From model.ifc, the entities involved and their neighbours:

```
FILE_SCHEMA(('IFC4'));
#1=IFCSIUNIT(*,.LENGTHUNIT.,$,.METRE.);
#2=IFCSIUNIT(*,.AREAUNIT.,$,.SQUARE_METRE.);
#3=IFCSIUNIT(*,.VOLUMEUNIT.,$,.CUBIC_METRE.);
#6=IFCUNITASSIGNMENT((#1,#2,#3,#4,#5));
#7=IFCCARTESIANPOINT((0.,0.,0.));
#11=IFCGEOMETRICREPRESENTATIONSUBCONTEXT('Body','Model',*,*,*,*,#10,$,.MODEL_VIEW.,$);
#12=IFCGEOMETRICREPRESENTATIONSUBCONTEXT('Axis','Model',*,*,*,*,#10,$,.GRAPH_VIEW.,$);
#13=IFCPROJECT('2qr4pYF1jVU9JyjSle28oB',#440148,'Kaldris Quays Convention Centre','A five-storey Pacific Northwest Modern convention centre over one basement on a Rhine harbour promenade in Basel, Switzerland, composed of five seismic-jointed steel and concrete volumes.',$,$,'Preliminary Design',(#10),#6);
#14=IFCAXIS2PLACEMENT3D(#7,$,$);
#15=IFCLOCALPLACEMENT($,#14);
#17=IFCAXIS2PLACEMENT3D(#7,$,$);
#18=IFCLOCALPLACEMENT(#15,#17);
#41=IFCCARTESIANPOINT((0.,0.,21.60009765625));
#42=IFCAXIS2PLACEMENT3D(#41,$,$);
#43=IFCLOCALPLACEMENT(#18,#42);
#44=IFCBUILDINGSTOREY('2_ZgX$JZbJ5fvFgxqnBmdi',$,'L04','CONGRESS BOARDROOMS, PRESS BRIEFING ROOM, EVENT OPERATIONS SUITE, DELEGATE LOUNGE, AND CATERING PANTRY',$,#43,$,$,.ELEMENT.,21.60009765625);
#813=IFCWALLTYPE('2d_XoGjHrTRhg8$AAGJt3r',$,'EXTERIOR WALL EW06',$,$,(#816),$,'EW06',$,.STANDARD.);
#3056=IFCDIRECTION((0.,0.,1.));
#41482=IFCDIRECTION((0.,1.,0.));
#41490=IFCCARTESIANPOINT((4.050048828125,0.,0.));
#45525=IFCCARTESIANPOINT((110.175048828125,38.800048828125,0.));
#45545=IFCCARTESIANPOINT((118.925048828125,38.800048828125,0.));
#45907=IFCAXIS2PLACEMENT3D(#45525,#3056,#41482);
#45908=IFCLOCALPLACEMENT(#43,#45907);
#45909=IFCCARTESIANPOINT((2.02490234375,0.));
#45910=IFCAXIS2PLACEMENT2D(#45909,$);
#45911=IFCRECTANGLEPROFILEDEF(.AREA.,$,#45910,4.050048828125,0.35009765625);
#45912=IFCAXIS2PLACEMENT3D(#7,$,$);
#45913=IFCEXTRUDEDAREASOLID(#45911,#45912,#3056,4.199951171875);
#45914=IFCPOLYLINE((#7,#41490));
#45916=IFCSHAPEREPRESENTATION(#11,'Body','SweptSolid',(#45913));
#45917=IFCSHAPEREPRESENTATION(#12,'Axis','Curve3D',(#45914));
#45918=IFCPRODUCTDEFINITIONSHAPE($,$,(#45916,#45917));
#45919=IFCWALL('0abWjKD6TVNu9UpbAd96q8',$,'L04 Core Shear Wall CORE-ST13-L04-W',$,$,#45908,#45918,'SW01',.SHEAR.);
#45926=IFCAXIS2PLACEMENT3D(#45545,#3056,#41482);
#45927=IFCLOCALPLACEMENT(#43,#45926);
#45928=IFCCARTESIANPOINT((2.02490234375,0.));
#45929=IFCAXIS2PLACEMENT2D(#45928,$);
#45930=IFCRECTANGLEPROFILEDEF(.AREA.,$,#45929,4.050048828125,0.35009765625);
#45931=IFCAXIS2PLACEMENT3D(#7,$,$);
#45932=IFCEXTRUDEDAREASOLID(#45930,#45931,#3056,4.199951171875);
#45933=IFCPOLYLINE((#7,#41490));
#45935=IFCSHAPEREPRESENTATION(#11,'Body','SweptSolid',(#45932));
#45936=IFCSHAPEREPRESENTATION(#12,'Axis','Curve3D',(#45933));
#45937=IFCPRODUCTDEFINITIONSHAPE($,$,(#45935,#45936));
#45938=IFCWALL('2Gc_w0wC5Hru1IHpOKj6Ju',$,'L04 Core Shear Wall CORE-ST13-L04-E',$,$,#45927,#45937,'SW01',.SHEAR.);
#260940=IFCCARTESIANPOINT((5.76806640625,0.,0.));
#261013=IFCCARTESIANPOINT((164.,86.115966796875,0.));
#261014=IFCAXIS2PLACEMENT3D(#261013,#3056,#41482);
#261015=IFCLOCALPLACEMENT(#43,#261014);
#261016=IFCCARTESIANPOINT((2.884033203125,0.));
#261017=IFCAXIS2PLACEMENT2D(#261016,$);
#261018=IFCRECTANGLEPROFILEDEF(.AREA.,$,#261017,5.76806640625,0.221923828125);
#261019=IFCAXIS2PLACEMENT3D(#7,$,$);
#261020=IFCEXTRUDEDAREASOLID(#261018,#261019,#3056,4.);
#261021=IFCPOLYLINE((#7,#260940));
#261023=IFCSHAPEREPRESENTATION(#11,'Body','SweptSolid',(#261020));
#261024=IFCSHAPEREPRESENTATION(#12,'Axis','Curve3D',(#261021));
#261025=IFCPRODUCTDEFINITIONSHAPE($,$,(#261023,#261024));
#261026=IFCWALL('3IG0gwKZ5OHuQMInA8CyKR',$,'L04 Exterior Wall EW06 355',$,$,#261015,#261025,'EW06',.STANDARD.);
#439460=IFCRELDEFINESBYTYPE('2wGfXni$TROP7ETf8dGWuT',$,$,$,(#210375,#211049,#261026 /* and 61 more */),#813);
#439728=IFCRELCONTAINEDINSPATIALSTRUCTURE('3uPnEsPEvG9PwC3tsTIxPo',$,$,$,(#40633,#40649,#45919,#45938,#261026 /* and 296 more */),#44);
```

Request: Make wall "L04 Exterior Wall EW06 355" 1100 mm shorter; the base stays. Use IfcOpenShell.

```python
import ifcopenshell
import ifcopenshell.geom
import ifcopenshell.util.representation
import ifcopenshell.util.shape

model = ifcopenshell.open("model.ifc")
settings = ifcopenshell.geom.settings()


def volume(element):
    """Net volume in cubic metres, openings subtracted."""
    shape = ifcopenshell.geom.create_shape(settings, element)
    return ifcopenshell.util.shape.get_volume(shape.geometry)


wall = model.by_guid("3IG0gwKZ5OHuQMInA8CyKR")
before = volume(wall)

body = ifcopenshell.util.representation.get_representation(wall, "Model", "Body")
solid = body.Items[0]
old_height = solid.Depth
solid.Depth -= 1.1
after = volume(wall)

print(f"height {old_height:g} -> {solid.Depth:g}, volume {before:.3f} -> {after:.3f} m3")

model.write("model_rev.ifc")
```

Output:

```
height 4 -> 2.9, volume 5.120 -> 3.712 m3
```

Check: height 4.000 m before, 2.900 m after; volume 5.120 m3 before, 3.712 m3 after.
